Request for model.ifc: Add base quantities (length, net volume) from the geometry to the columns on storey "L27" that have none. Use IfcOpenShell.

First a look at what the model holds.

```python
import ifcopenshell
import ifcopenshell.util.element
import ifcopenshell.util.unit

model = ifcopenshell.open("model.ifc")
print(model.schema)
for unit_type in ("LENGTHUNIT", "AREAUNIT", "VOLUMEUNIT"):
    print(unit_type, ifcopenshell.util.unit.calculate_unit_scale(model, unit_type))
storey = next(s for s in model.by_type("IfcBuildingStorey") if s.Name == "L27")
columns = [e for e in ifcopenshell.util.element.get_decomposition(storey) if e.is_a("IfcColumn")]
for e in sorted(columns, key=lambda e: e.id()):
    print(e.id(), e.is_a(), e.Name, list(ifcopenshell.util.element.get_psets(e, qtos_only=True)), sep=" | ")
```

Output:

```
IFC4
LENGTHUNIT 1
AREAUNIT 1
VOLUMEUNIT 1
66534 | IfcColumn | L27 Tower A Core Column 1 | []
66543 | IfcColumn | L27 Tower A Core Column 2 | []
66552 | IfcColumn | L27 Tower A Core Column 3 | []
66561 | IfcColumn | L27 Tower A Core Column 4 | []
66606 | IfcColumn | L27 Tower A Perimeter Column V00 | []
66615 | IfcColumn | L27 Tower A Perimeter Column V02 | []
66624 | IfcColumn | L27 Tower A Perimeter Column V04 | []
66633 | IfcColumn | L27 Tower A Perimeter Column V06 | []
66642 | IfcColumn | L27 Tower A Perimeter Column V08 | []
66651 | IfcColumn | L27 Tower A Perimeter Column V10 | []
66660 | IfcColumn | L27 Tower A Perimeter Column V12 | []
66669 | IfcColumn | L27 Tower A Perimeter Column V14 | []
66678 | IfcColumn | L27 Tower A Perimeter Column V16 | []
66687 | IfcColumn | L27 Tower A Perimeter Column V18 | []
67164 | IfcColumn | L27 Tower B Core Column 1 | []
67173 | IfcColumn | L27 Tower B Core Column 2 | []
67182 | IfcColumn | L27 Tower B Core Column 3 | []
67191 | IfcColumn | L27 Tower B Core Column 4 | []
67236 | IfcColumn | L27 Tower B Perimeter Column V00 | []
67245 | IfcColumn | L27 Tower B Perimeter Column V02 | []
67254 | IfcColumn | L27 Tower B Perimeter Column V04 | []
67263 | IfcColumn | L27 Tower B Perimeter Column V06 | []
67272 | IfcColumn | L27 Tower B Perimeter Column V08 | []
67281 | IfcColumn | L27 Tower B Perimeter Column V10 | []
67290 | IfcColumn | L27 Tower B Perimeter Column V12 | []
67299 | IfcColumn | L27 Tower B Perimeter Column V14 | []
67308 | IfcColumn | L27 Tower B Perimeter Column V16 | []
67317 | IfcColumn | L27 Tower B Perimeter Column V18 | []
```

```python
import ifcopenshell
import ifcopenshell.api.pset
import ifcopenshell.geom
import ifcopenshell.util.element
import ifcopenshell.util.shape
import ifcopenshell.util.unit

model = ifcopenshell.open("model.ifc")
unit_scale = ifcopenshell.util.unit.calculate_unit_scale(model)
volume_scale = ifcopenshell.util.unit.calculate_unit_scale(model, "VOLUMEUNIT")
settings = ifcopenshell.geom.settings()

storey = next(s for s in model.by_type("IfcBuildingStorey") if s.Name == "L27")
columns = [e for e in ifcopenshell.util.element.get_decomposition(storey) if e.is_a("IfcColumn")]

for e in sorted(columns, key=lambda e: e.id()):
    if ifcopenshell.util.element.get_psets(e, qtos_only=True, should_inherit=False):
        continue
    # Geometry comes back in metres, in the element's own axes.
    shape = ifcopenshell.geom.create_shape(settings, e)
    values = {
        "Length": ifcopenshell.util.shape.get_z(shape.geometry) / unit_scale,
        "NetVolume": ifcopenshell.util.shape.get_volume(shape.geometry) / volume_scale,
    }
    qto = ifcopenshell.api.pset.add_qto(model, product=e, name="Qto_ColumnBaseQuantities")
    ifcopenshell.api.pset.edit_qto(model, qto=qto, properties=values)
    print(e.id(), {k: round(v, 3) for k, v in values.items()})

model.write("model-out.ifc")
```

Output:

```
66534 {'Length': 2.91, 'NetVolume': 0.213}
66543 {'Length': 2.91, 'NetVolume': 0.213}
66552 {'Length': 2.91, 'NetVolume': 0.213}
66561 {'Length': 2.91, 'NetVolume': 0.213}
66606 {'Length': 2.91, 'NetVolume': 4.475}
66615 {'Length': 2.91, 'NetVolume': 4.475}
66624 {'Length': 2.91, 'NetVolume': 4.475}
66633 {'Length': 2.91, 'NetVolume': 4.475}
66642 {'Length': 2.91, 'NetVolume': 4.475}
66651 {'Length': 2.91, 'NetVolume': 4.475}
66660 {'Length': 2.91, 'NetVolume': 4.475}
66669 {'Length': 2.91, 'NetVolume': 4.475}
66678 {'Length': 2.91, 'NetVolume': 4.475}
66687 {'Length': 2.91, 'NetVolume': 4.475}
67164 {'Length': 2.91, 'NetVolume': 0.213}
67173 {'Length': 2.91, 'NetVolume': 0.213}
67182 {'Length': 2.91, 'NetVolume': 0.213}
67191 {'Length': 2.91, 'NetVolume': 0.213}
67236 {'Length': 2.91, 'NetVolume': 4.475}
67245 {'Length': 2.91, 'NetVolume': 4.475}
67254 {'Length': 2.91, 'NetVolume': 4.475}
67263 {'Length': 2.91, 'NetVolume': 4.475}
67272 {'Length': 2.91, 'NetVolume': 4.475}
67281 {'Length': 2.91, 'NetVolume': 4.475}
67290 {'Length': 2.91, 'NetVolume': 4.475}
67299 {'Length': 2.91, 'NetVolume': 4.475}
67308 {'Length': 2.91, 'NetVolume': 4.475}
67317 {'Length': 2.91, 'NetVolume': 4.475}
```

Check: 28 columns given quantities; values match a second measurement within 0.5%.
